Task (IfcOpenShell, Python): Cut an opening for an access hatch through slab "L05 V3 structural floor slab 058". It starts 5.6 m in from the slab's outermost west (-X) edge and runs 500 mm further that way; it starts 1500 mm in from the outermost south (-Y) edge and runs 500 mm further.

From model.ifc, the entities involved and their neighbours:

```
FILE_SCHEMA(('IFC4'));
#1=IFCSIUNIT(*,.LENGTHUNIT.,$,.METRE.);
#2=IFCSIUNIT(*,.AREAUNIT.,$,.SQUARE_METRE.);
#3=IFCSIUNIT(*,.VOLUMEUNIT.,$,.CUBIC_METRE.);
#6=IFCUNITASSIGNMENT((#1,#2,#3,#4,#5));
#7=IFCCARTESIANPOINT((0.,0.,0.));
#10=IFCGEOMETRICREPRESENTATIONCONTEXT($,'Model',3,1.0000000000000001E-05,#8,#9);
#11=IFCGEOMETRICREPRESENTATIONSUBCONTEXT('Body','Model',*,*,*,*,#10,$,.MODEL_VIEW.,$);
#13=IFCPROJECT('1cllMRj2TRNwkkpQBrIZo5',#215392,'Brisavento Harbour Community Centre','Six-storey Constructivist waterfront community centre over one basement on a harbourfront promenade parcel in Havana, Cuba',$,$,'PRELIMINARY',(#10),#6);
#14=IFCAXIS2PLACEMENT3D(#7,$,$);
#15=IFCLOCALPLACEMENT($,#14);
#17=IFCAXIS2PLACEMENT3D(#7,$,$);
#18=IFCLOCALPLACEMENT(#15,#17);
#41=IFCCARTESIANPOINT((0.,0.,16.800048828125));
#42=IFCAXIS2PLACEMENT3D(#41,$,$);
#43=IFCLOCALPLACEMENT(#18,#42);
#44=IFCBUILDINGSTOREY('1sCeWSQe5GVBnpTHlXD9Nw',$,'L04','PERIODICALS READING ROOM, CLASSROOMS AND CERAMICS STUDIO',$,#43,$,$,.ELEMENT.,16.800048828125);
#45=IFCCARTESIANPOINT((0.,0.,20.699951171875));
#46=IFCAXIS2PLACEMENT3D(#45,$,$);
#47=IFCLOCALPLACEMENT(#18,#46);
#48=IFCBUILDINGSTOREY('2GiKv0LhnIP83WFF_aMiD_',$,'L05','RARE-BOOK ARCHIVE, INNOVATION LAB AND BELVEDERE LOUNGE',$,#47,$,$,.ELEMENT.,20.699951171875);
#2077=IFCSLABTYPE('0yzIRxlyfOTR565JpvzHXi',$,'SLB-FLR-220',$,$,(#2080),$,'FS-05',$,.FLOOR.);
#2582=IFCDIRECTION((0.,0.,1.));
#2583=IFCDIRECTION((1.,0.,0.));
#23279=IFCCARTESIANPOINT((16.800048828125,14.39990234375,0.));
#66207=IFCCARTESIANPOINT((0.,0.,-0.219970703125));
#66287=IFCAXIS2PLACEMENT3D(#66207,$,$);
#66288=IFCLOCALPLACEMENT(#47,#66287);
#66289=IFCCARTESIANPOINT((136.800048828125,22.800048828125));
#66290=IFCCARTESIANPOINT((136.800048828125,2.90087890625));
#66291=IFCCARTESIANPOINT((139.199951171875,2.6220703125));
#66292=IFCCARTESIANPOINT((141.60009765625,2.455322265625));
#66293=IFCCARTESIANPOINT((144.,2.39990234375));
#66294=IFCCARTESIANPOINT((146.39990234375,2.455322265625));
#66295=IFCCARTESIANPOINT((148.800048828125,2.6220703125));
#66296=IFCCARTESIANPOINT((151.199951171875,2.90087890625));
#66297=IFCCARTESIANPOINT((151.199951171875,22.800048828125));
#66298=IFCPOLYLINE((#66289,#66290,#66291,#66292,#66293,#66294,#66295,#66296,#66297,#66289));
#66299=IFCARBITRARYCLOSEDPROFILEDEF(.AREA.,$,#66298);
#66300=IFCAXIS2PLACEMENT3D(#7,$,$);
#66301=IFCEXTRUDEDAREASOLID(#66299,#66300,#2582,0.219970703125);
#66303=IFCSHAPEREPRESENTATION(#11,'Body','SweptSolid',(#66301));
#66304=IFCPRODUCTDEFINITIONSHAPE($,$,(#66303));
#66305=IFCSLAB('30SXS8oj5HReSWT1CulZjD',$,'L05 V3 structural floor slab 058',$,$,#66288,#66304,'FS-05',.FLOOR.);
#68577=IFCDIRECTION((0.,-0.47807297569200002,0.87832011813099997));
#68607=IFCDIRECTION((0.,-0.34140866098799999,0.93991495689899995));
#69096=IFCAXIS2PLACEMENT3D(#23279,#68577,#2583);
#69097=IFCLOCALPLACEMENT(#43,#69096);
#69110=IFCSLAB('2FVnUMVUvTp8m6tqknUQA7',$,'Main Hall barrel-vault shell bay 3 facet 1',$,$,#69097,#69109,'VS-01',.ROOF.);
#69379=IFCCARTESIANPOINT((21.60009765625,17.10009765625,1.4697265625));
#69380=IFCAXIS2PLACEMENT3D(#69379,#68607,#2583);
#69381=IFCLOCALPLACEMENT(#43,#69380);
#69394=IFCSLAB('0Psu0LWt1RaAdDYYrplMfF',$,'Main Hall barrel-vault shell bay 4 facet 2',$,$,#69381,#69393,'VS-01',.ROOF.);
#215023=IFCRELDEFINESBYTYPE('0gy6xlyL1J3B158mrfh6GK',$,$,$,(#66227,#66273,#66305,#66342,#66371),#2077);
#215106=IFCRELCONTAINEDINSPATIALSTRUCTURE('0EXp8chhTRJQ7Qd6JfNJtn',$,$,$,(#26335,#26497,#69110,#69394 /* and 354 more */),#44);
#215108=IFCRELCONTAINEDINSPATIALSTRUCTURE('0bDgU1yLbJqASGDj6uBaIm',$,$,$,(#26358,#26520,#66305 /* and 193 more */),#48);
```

```python
import numpy as np
import ifcopenshell
import ifcopenshell.api.feature
import ifcopenshell.api.geometry
import ifcopenshell.api.root
import ifcopenshell.geom
import ifcopenshell.util.placement
import ifcopenshell.util.representation
import ifcopenshell.util.shape
import ifcopenshell.util.unit

model = ifcopenshell.open("model.ifc")
unit_scale = ifcopenshell.util.unit.calculate_unit_scale(model)
settings = ifcopenshell.geom.settings()


def volume(element):
    """Net volume in cubic metres, openings subtracted."""
    shape = ifcopenshell.geom.create_shape(settings, element)
    return ifcopenshell.util.shape.get_volume(shape.geometry)


slab = model.by_guid("30SXS8oj5HReSWT1CulZjD")
before = volume(slab)

# Extent in the slab's own axes, in metres. The edges named are its -X and -Y sides.
slab_shape = ifcopenshell.geom.create_shape(settings, slab)
vertices = ifcopenshell.util.shape.get_vertices(slab_shape.geometry)
x_min, y_min, bottom = vertices.min(axis=0)
top = vertices[:, 2].max()

opening = ifcopenshell.api.root.create_entity(model, ifc_class="IfcOpeningElement", name="Access hatch opening", predefined_type="OPENING")
context = ifcopenshell.util.representation.get_context(model, "Model", "Body", "MODEL_VIEW")
width, depth = 0.5, 0.5
outline = [(0.0, 0.0), (width, 0.0), (width, depth), (0.0, depth), (0.0, 0.0)]
# Overshoot both faces by 50 mm so the cut is clean.
shape = ifcopenshell.api.geometry.add_slab_representation(
    model, context=context, depth=top - bottom + 0.1, polyline=outline
)
ifcopenshell.api.geometry.assign_representation(model, product=opening, representation=shape)

matrix = ifcopenshell.util.placement.get_local_placement(slab.ObjectPlacement)
matrix[:, 3] = matrix @ np.append(np.array([x_min + 5.6, y_min + 1.5, bottom - 0.05]) / unit_scale, 1.0)
ifcopenshell.api.geometry.edit_object_placement(model, product=opening, matrix=matrix, is_si=False)
ifcopenshell.api.feature.add_feature(model, feature=opening, element=slab)

after = volume(slab)

print(f"slab volume {before:.3f} -> {after:.3f} m3")

model.write("model_rev.ifc")
```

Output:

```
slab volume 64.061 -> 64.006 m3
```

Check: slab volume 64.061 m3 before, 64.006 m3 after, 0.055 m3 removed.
